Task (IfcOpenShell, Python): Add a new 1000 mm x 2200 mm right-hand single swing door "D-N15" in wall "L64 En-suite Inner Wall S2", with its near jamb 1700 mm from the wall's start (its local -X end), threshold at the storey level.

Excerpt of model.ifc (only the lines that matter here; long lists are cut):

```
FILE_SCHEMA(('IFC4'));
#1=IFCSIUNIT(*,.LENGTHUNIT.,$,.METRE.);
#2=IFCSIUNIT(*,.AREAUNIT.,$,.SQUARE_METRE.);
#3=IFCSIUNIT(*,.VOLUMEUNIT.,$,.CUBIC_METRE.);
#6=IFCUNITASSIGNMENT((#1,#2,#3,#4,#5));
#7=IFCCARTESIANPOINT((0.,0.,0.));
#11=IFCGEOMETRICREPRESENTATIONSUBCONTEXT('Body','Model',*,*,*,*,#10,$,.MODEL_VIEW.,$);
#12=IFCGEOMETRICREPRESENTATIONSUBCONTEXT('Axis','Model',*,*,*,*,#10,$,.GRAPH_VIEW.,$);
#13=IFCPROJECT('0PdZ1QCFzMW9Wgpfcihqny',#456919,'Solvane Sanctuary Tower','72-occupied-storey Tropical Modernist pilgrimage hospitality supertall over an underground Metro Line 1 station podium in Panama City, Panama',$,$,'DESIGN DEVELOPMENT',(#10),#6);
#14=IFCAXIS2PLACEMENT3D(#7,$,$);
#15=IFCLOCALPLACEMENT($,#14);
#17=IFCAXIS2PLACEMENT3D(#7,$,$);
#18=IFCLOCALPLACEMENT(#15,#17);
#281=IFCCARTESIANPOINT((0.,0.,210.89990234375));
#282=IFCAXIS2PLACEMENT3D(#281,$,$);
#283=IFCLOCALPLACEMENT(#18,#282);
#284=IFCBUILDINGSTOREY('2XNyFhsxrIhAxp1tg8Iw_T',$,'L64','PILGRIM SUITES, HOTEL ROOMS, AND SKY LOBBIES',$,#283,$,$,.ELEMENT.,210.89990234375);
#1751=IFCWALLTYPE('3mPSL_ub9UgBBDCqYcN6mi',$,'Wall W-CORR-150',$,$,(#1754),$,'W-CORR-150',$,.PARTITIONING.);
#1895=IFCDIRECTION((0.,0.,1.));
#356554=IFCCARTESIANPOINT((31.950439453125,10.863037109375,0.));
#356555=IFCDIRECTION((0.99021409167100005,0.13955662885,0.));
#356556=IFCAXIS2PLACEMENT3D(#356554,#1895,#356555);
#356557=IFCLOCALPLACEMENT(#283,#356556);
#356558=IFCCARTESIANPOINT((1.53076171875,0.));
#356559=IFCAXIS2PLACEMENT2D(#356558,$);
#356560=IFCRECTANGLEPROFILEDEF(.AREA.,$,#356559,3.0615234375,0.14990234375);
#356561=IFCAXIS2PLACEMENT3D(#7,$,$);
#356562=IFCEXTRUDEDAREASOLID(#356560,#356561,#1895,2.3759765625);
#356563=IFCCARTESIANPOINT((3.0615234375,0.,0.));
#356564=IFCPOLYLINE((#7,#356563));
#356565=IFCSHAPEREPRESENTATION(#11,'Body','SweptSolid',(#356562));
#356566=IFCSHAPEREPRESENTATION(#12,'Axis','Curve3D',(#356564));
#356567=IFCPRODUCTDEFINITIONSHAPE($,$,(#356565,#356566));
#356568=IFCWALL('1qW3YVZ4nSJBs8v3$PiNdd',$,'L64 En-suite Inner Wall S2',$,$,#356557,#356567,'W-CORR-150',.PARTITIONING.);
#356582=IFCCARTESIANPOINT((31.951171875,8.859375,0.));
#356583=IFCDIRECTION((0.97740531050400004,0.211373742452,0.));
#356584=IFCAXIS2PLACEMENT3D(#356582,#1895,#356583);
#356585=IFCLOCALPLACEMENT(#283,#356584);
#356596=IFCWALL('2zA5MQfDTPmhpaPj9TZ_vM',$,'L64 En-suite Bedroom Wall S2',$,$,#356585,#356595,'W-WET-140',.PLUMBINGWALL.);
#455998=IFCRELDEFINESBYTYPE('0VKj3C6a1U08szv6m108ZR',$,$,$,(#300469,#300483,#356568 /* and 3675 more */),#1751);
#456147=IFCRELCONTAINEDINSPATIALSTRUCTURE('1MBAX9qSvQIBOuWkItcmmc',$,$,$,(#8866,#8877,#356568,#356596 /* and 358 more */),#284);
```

```python
import numpy as np
import ifcopenshell
import ifcopenshell.api.feature
import ifcopenshell.api.geometry
import ifcopenshell.api.root
import ifcopenshell.api.spatial
import ifcopenshell.geom
import ifcopenshell.util.element
import ifcopenshell.util.placement
import ifcopenshell.util.representation
import ifcopenshell.util.shape
import ifcopenshell.util.unit

model = ifcopenshell.open("model.ifc")
unit_scale = ifcopenshell.util.unit.calculate_unit_scale(model)
settings = ifcopenshell.geom.settings()


def volume(element):
    """Net volume in cubic metres, openings subtracted."""
    shape = ifcopenshell.geom.create_shape(settings, element)
    return ifcopenshell.util.shape.get_volume(shape.geometry)


wall = model.by_guid("1qW3YVZ4nSJBs8v3$PiNdd")
storey = ifcopenshell.util.element.get_container(wall, ifc_class="IfcBuildingStorey")
context = ifcopenshell.util.representation.get_context(model, "Model", "Body", "MODEL_VIEW")
before = volume(wall)

width, height, from_end, sill = 1, 2.2, 1.7, 0.0  # metres

# The wall runs along its own X axis, and the end named is its -X end.
wall_shape = ifcopenshell.geom.create_shape(settings, wall)
x, y, z = ifcopenshell.util.shape.get_vertices(wall_shape.geometry).T
start = x.min() + from_end
face, thickness = float(y.min()), float(y.max() - y.min())
wall_matrix = ifcopenshell.util.placement.get_local_placement(wall.ObjectPlacement)
level = ifcopenshell.util.placement.get_local_placement(storey.ObjectPlacement)[2, 3]


def in_wall(x, y):
    """Placement at x, y metres in the wall's axes, at sill height."""
    matrix = wall_matrix.copy()
    matrix[:, 3] = wall_matrix @ np.array([x / unit_scale, y / unit_scale, 0.0, 1.0])
    matrix[2, 3] = level + sill / unit_scale
    return matrix


# Opening: a box that overshoots both wall faces by 50 mm.
opening = ifcopenshell.api.root.create_entity(model, ifc_class="IfcOpeningElement", predefined_type="OPENING")
box = ifcopenshell.api.geometry.add_wall_representation(
    model, context=context, length=width, height=height, thickness=thickness + 0.1
)
ifcopenshell.api.geometry.assign_representation(model, product=opening, representation=box)
ifcopenshell.api.geometry.edit_object_placement(model, product=opening, matrix=in_wall(start, face - 0.05), is_si=False)
ifcopenshell.api.feature.add_feature(model, feature=opening, element=wall)

door = ifcopenshell.api.root.create_entity(model, ifc_class="IfcDoor", name="D-N15", predefined_type="DOOR")
door.OverallWidth, door.OverallHeight = width / unit_scale, height / unit_scale
door.OperationType = "SINGLE_SWING_RIGHT"
body = ifcopenshell.api.geometry.add_door_representation(
    model,
    context=context,
    overall_width=door.OverallWidth,
    overall_height=door.OverallHeight,
    operation_type="SINGLE_SWING_RIGHT",
    lining_properties={"LiningDepth": thickness / unit_scale, "ThresholdDepth": thickness / unit_scale},
)
ifcopenshell.api.geometry.assign_representation(model, product=door, representation=body)
ifcopenshell.api.spatial.assign_container(model, products=[door], relating_structure=storey)
ifcopenshell.api.feature.add_filling(model, opening=opening, element=door)

# The lining spans the wall, so the door starts at the wall face.
ifcopenshell.api.geometry.edit_object_placement(model, product=door, matrix=in_wall(start, face), is_si=False)

after = volume(wall)

print(f"wall volume {before:.3f} -> {after:.3f} m3")

model.write("model_edited.ifc")
```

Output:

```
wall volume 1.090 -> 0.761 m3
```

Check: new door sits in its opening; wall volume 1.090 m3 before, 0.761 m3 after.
